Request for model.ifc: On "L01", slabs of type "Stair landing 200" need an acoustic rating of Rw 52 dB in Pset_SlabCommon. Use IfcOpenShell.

First a look at what the model holds.

```python
import ifcopenshell
import ifcopenshell.util.element

model = ifcopenshell.open("model.ifc")
print(model.schema)
storey = next(s for s in model.by_type("IfcBuildingStorey") if s.Name == "L01")
slabs = [e for e in ifcopenshell.util.element.get_decomposition(storey) if e.is_a("IfcSlab")]
seen = {}
for e in slabs:
    element_type = ifcopenshell.util.element.get_type(e)
    key = (element_type.Name if element_type != e and element_type else None, ifcopenshell.util.element.get_pset(e, "Pset_SlabCommon", "AcousticRating"))
    seen[key] = seen.get(key, 0) + 1
for (name, value), count in sorted(seen.items(), key=str):
    print(count, "x", name, "|", value)
```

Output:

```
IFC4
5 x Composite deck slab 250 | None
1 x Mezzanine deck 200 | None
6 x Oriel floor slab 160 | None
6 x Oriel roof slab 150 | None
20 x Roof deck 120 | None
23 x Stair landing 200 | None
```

```python
import ifcopenshell
import ifcopenshell.api.pset
import ifcopenshell.util.element

model = ifcopenshell.open("model.ifc")

storey = next(s for s in model.by_type("IfcBuildingStorey") if s.Name == "L01")
slabs = [e for e in ifcopenshell.util.element.get_decomposition(storey) if e.is_a("IfcSlab")]

count = 0
for e in slabs:
    element_type = ifcopenshell.util.element.get_type(e)
    if element_type in (None, e) or element_type.Name != "Stair landing 200":
        continue
    # add_pset returns the element's existing set when there is one.
    pset = ifcopenshell.api.pset.add_pset(model, product=e, name="Pset_SlabCommon")
    ifcopenshell.api.pset.edit_pset(model, pset=pset, properties={"AcousticRating": "Rw 52 dB"})
    count += 1

print(count, "slabs updated")

model.write("model_rev.ifc")
```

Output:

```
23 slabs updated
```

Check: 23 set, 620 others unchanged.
